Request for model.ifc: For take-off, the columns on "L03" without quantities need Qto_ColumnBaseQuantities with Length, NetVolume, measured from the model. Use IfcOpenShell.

First a look at what the model holds.

```python
import ifcopenshell
import ifcopenshell.util.element
import ifcopenshell.util.unit

model = ifcopenshell.open("model.ifc")
print(model.schema)
for unit_type in ("LENGTHUNIT", "AREAUNIT", "VOLUMEUNIT"):
    print(unit_type, ifcopenshell.util.unit.calculate_unit_scale(model, unit_type))
storey = next(s for s in model.by_type("IfcBuildingStorey") if s.Name == "L03")
columns = [e for e in ifcopenshell.util.element.get_decomposition(storey) if e.is_a("IfcColumn")]
for e in sorted(columns, key=lambda e: e.id()):
    print(e.id(), e.is_a(), e.Name, list(ifcopenshell.util.element.get_psets(e, qtos_only=True)), sep=" | ")
```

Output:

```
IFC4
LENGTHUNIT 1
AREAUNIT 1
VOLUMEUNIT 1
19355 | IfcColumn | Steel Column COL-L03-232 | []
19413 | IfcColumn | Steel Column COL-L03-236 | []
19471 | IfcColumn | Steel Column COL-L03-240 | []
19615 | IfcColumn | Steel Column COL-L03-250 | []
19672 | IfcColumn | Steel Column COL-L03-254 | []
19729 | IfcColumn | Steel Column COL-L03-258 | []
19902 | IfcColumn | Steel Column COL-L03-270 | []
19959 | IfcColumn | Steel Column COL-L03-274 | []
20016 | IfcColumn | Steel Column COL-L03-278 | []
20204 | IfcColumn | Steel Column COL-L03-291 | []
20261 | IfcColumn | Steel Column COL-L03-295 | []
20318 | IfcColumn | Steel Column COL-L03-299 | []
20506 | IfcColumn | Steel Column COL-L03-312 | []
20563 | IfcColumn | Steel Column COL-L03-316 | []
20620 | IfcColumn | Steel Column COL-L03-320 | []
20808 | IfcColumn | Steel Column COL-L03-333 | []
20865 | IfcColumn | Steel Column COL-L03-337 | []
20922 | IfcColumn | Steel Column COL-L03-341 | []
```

```python
import ifcopenshell
import ifcopenshell.api.pset
import ifcopenshell.geom
import ifcopenshell.util.element
import ifcopenshell.util.shape
import ifcopenshell.util.unit

model = ifcopenshell.open("model.ifc")
unit_scale = ifcopenshell.util.unit.calculate_unit_scale(model)
volume_scale = ifcopenshell.util.unit.calculate_unit_scale(model, "VOLUMEUNIT")
settings = ifcopenshell.geom.settings()

storey = next(s for s in model.by_type("IfcBuildingStorey") if s.Name == "L03")
columns = [e for e in ifcopenshell.util.element.get_decomposition(storey) if e.is_a("IfcColumn")]

for e in sorted(columns, key=lambda e: e.id()):
    if ifcopenshell.util.element.get_psets(e, qtos_only=True, should_inherit=False):
        continue
    # Geometry comes back in metres, in the element's own axes.
    shape = ifcopenshell.geom.create_shape(settings, e)
    values = {
        "Length": ifcopenshell.util.shape.get_z(shape.geometry) / unit_scale,
        "NetVolume": ifcopenshell.util.shape.get_volume(shape.geometry) / volume_scale,
    }
    qto = ifcopenshell.api.pset.add_qto(model, product=e, name="Qto_ColumnBaseQuantities")
    ifcopenshell.api.pset.edit_qto(model, qto=qto, properties=values)
    print(e.id(), {k: round(v, 3) for k, v in values.items()})

model.write("model_v2.ifc")
```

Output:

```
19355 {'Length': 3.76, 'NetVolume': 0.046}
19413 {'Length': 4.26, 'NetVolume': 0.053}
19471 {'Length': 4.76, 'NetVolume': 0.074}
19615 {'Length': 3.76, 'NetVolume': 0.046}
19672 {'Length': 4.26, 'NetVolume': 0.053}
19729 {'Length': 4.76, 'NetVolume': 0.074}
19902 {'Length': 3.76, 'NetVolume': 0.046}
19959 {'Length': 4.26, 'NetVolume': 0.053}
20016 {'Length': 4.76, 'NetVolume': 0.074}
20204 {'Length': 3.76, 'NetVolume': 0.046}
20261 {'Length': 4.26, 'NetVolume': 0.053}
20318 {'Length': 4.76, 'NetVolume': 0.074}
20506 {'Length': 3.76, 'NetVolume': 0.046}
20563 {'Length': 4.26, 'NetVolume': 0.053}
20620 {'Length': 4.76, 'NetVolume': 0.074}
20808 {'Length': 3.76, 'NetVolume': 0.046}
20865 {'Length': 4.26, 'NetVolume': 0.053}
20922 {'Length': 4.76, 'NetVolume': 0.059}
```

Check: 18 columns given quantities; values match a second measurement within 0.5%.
